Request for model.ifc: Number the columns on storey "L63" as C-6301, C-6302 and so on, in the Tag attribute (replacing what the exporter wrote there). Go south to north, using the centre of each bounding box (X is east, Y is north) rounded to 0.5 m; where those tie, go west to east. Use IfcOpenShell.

First a look at what the model holds.

```python
import ifcopenshell
import ifcopenshell.util.element
import ifcopenshell.util.placement

model = ifcopenshell.open("model.ifc")
print(model.schema)
storey = next(s for s in model.by_type("IfcBuildingStorey") if s.Name == "L63")
columns = [e for e in ifcopenshell.util.element.get_decomposition(storey) if e.is_a("IfcColumn")]
for e in sorted(columns, key=lambda e: e.id()):
    origin = ifcopenshell.util.placement.get_local_placement(e.ObjectPlacement)[:3, 3]
    print(e.id(), e.Tag, e.Name, origin.round(2) + 0.0, sep=" | ")
```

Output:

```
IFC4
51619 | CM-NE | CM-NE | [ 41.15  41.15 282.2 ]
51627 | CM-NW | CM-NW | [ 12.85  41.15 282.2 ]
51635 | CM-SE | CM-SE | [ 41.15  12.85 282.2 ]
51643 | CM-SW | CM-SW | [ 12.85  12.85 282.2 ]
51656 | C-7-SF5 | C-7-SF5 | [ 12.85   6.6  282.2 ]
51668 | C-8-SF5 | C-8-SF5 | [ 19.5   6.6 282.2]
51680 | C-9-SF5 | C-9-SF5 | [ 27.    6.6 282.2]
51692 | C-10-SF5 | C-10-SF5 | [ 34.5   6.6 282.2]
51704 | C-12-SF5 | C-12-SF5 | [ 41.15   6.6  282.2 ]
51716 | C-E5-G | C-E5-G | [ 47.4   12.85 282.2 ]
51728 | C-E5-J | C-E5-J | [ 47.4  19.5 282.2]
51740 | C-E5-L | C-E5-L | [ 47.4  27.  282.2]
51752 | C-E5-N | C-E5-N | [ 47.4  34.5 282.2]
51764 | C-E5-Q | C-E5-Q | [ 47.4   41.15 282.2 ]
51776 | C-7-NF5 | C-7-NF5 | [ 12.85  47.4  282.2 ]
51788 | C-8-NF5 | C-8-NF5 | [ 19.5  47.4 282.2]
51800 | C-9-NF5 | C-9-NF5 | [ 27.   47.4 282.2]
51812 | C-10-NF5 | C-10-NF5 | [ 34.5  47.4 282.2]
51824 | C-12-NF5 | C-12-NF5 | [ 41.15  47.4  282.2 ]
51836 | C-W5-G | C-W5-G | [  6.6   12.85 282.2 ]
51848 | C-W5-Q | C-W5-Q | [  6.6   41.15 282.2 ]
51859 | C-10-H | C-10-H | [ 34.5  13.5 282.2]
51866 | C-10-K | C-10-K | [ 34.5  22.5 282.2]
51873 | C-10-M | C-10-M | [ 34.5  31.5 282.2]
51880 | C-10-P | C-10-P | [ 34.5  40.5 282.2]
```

```python
import ifcopenshell
import ifcopenshell.geom
import ifcopenshell.util.element
import ifcopenshell.util.shape

model = ifcopenshell.open("model.ifc")
settings = ifcopenshell.geom.settings()
settings.set("use-world-coords", True)


def centre(element):
    shape = ifcopenshell.geom.create_shape(settings, element)
    return ifcopenshell.util.shape.get_bbox_centroid(shape.geometry)


storey = next(s for s in model.by_type("IfcBuildingStorey") if s.Name == "L63")
columns = [e for e in ifcopenshell.util.element.get_decomposition(storey) if e.is_a("IfcColumn")]

# Insertion points can sit at a corner or the storey origin, so sort by the geometry (in metres).
centres = {e: centre(e) for e in columns}
columns.sort(key=lambda e: (round(centres[e][1] / 0.5), centres[e][0]))

for i, e in enumerate(columns, start=1):
    number = f"C-63{i:02d}"
    e.Tag = number
    print(e.id(), number)

model.write("model-out.ifc")
```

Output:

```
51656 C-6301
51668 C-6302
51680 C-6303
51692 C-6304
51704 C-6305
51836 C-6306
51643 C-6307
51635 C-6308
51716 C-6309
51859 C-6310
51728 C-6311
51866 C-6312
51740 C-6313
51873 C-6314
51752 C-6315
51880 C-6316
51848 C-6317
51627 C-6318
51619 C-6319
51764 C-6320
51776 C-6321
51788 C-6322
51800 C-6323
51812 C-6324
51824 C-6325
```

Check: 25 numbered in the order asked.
